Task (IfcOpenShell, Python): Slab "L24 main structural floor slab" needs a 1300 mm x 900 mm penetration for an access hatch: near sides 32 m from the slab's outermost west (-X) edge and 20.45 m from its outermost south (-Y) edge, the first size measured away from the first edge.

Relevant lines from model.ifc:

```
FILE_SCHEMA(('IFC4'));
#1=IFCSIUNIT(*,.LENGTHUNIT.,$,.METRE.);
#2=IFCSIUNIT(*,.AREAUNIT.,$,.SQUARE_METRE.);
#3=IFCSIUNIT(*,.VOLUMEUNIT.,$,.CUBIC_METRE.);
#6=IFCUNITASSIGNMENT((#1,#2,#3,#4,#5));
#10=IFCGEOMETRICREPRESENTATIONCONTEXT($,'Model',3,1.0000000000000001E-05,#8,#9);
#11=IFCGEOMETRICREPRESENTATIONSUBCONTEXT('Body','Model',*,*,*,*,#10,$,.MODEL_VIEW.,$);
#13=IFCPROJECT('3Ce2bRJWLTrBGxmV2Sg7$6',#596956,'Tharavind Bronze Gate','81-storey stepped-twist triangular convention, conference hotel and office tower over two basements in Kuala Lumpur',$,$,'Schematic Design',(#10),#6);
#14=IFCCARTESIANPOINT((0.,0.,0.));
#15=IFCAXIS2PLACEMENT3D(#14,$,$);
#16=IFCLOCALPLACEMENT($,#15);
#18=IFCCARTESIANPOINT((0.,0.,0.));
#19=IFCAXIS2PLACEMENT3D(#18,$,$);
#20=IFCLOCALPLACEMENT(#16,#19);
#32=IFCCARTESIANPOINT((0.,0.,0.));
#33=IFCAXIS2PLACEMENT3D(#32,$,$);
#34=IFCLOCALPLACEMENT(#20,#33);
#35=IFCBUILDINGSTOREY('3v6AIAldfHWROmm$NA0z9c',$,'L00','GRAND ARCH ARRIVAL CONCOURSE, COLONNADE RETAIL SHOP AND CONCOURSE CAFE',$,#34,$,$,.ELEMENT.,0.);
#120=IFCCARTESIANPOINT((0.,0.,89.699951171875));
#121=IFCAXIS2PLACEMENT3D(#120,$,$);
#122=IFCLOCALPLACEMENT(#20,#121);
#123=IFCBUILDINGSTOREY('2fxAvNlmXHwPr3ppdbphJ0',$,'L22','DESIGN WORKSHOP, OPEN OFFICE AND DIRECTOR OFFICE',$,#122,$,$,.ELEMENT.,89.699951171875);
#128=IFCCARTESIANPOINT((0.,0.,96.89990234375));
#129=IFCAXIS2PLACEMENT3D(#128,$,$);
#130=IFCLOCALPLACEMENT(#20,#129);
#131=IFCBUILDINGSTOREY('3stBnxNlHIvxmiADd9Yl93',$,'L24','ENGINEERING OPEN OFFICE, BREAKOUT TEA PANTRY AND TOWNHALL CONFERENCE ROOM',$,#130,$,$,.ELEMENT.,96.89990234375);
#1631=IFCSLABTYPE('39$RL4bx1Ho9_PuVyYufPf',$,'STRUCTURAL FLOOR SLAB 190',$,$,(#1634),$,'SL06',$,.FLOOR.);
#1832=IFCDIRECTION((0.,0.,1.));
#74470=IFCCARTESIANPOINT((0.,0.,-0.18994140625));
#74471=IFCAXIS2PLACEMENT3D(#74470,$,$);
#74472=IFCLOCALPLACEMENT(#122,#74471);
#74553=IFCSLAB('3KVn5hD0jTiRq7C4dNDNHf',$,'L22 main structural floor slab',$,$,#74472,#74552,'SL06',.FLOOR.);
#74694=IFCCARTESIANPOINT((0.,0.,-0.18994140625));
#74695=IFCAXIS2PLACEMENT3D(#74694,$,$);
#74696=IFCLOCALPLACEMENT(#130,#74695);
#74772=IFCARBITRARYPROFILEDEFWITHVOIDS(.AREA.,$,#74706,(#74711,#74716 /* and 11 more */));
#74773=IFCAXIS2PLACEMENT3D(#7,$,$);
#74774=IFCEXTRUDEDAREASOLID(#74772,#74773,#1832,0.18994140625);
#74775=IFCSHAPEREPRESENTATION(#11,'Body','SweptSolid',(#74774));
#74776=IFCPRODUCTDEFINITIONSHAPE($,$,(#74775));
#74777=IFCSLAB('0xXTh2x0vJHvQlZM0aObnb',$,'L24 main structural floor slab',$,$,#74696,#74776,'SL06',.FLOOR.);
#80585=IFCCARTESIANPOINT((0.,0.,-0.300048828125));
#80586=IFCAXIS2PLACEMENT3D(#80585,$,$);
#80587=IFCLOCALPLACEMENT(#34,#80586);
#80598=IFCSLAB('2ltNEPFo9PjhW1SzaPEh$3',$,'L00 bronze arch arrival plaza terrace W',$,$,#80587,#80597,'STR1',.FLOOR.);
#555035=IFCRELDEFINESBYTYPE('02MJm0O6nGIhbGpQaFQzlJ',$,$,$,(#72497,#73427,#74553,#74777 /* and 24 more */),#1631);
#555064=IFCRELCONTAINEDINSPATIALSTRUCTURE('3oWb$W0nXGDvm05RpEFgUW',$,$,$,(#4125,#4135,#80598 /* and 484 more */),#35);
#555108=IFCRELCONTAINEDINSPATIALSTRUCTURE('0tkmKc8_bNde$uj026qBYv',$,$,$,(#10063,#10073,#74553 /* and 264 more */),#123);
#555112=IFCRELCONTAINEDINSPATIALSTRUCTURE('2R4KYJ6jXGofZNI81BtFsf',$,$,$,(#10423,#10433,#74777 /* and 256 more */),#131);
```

```python
import numpy as np
import ifcopenshell
import ifcopenshell.api.feature
import ifcopenshell.api.geometry
import ifcopenshell.api.root
import ifcopenshell.geom
import ifcopenshell.util.placement
import ifcopenshell.util.representation
import ifcopenshell.util.shape
import ifcopenshell.util.unit

model = ifcopenshell.open("model.ifc")
unit_scale = ifcopenshell.util.unit.calculate_unit_scale(model)
settings = ifcopenshell.geom.settings()


def volume(element):
    """Net volume in cubic metres, openings subtracted."""
    shape = ifcopenshell.geom.create_shape(settings, element)
    return ifcopenshell.util.shape.get_volume(shape.geometry)


slab = model.by_guid("0xXTh2x0vJHvQlZM0aObnb")
before = volume(slab)

# Extent in the slab's own axes, in metres. The edges named are its -X and -Y sides.
slab_shape = ifcopenshell.geom.create_shape(settings, slab)
vertices = ifcopenshell.util.shape.get_vertices(slab_shape.geometry)
x_min, y_min, bottom = vertices.min(axis=0)
top = vertices[:, 2].max()

opening = ifcopenshell.api.root.create_entity(model, ifc_class="IfcOpeningElement", name="Access hatch opening", predefined_type="OPENING")
context = ifcopenshell.util.representation.get_context(model, "Model", "Body", "MODEL_VIEW")
width, depth = 1.3, 0.9
outline = [(0.0, 0.0), (width, 0.0), (width, depth), (0.0, depth), (0.0, 0.0)]
# Overshoot both faces by 50 mm so the cut is clean.
shape = ifcopenshell.api.geometry.add_slab_representation(
    model, context=context, depth=top - bottom + 0.1, polyline=outline
)
ifcopenshell.api.geometry.assign_representation(model, product=opening, representation=shape)

matrix = ifcopenshell.util.placement.get_local_placement(slab.ObjectPlacement)
matrix[:, 3] = matrix @ np.append(np.array([x_min + 32, y_min + 20.45, bottom - 0.05]) / unit_scale, 1.0)
ifcopenshell.api.geometry.edit_object_placement(model, product=opening, matrix=matrix, is_si=False)
ifcopenshell.api.feature.add_feature(model, feature=opening, element=slab)

after = volume(slab)

print(f"slab volume {before:.3f} -> {after:.3f} m3")

model.write("model_v2.ifc")
```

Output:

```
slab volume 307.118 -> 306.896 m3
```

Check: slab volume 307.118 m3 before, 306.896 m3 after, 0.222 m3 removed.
